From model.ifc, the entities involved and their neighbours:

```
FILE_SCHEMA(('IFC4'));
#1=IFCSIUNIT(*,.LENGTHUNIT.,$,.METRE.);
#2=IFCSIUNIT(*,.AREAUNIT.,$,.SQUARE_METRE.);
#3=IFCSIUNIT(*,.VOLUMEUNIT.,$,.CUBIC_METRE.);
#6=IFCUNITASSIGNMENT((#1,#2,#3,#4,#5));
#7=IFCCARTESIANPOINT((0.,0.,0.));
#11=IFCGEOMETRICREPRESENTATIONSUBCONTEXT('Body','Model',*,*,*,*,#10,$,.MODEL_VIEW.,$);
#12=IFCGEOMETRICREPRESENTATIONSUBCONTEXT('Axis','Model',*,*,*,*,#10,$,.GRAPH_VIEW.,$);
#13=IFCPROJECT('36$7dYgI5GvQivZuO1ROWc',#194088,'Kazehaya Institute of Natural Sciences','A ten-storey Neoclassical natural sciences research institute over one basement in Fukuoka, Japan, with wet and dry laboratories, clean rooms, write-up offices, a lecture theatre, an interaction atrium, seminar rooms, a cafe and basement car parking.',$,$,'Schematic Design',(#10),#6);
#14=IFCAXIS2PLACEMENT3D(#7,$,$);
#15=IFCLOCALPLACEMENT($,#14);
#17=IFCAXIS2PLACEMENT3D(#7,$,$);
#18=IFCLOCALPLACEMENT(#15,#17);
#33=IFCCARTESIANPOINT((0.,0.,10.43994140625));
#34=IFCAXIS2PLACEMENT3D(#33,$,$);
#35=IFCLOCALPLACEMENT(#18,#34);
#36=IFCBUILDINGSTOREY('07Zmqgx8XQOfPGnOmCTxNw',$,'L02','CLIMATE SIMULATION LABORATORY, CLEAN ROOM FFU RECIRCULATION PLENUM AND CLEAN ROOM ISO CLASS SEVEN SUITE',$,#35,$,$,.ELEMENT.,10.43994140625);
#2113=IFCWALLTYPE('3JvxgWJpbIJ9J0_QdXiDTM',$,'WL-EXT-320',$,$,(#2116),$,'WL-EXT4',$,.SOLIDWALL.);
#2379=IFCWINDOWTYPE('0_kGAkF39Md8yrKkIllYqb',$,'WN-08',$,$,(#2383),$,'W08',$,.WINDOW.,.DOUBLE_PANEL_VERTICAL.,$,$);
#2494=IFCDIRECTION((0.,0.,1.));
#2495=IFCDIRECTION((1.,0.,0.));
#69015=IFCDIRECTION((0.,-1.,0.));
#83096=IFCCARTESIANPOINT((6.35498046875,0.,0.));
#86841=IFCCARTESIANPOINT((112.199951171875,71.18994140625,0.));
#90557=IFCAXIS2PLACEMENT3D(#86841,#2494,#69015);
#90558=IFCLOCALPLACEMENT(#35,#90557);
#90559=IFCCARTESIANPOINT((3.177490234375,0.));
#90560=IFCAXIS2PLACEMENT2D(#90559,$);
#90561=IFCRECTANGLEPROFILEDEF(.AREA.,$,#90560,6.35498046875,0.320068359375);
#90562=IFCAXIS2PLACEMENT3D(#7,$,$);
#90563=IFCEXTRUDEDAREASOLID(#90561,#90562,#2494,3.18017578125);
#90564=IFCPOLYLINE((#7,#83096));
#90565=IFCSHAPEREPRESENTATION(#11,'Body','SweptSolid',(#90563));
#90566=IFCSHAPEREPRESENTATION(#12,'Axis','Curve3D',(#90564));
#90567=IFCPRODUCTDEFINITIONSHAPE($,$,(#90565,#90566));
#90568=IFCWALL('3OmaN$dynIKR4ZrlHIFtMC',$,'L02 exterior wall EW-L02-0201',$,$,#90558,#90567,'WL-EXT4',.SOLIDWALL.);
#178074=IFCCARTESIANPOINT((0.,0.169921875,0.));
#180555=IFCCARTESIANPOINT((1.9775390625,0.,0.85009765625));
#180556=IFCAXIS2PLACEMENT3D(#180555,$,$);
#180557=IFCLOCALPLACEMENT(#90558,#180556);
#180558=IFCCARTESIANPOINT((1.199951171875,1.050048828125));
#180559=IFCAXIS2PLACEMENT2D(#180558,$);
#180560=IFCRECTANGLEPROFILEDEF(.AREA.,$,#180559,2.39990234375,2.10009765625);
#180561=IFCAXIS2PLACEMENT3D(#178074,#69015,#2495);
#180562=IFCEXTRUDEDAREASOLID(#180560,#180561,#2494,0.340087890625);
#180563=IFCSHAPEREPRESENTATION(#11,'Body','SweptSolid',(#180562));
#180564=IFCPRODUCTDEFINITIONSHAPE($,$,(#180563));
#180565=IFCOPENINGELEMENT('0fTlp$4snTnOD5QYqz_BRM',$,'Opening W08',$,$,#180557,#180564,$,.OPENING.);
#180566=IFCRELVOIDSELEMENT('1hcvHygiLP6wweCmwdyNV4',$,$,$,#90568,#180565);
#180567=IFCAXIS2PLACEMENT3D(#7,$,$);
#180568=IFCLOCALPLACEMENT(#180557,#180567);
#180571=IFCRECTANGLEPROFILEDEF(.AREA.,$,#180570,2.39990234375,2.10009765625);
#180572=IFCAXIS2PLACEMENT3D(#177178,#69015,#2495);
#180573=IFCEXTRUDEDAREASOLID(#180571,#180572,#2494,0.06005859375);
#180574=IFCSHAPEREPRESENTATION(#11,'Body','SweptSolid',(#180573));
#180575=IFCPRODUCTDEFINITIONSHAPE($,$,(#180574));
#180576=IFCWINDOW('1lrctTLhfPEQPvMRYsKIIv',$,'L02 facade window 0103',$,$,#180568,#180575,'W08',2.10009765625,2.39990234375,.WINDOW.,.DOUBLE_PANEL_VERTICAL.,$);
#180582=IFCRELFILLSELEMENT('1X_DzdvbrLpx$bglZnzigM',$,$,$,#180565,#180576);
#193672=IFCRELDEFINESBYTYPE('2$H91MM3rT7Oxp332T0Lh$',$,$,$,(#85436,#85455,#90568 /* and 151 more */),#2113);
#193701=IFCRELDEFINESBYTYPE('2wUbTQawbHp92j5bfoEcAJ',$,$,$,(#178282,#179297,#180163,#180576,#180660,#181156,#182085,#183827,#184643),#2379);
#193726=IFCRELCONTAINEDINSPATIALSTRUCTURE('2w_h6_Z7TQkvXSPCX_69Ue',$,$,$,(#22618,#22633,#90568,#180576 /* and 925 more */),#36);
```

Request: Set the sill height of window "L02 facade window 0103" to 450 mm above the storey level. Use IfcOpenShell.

```python
import numpy as np
import ifcopenshell
import ifcopenshell.api.geometry
import ifcopenshell.geom
import ifcopenshell.util.element
import ifcopenshell.util.placement
import ifcopenshell.util.shape
import ifcopenshell.util.unit

model = ifcopenshell.open("model.ifc")
unit_scale = ifcopenshell.util.unit.calculate_unit_scale(model)

window = model.by_guid("1lrctTLhfPEQPvMRYsKIIv")
opening = window.FillsVoids[0].RelatingOpeningElement
storey = ifcopenshell.util.element.get_container(window, ifc_class="IfcBuildingStorey")
level = ifcopenshell.util.placement.get_local_placement(storey.ObjectPlacement)[2, 3]

# The opening's origin need not be at the sill, so measure its lowest point.
shape = ifcopenshell.geom.create_shape(ifcopenshell.geom.settings(), opening)
bottom = ifcopenshell.util.shape.get_shape_bottom_elevation(shape, shape.geometry) / unit_scale
dz = level + 0.45 / unit_scale - bottom

shift = np.array([0.0, 0.0, dz])
# The window is placed relative to its opening, so it follows when the opening moves.
matrix = ifcopenshell.util.placement.get_local_placement(opening.ObjectPlacement)
matrix[:3, 3] += shift
ifcopenshell.api.geometry.edit_object_placement(
    model, product=opening, matrix=matrix, is_si=False, should_transform_children=True
)

print(f"moved by {dz * unit_scale:+.3f} m")

model.write("model-out.ifc")
```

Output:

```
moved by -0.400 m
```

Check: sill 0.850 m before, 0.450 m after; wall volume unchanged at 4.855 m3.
